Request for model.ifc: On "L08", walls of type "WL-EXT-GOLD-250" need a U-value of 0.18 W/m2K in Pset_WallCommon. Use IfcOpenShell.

First a look at what the model holds.

```python
import ifcopenshell
import ifcopenshell.util.element

model = ifcopenshell.open("model.ifc")
print(model.schema)
storey = next(s for s in model.by_type("IfcBuildingStorey") if s.Name == "L08")
walls = [e for e in ifcopenshell.util.element.get_decomposition(storey) if e.is_a("IfcWall")]
seen = {}
for e in walls:
    element_type = ifcopenshell.util.element.get_type(e)
    key = (element_type.Name if element_type != e and element_type else None, ifcopenshell.util.element.get_pset(e, "Pset_WallCommon", "ThermalTransmittance"))
    seen[key] = seen.get(key, 0) + 1
for (name, value), count in sorted(seen.items(), key=str):
    print(count, "x", name, "|", value)
```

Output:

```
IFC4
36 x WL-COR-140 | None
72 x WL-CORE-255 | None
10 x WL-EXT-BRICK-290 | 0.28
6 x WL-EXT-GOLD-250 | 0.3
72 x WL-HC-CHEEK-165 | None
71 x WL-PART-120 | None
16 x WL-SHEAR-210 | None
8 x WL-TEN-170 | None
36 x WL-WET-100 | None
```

```python
import ifcopenshell
import ifcopenshell.api.pset
import ifcopenshell.util.element

model = ifcopenshell.open("model.ifc")

storey = next(s for s in model.by_type("IfcBuildingStorey") if s.Name == "L08")
walls = [e for e in ifcopenshell.util.element.get_decomposition(storey) if e.is_a("IfcWall")]

count = 0
for e in walls:
    element_type = ifcopenshell.util.element.get_type(e)
    if element_type in (None, e) or element_type.Name != "WL-EXT-GOLD-250":
        continue
    # add_pset returns the element's existing set when there is one.
    pset = ifcopenshell.api.pset.add_pset(model, product=e, name="Pset_WallCommon")
    ifcopenshell.api.pset.edit_pset(model, pset=pset, properties={"ThermalTransmittance": 0.18})
    count += 1

print(count, "walls updated")

model.write("model_rev.ifc")
```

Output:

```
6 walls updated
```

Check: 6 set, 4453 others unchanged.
